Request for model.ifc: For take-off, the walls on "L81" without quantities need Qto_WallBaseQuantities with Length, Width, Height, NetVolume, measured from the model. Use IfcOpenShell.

First a look at what the model holds.

```python
import ifcopenshell
import ifcopenshell.util.element
import ifcopenshell.util.unit

model = ifcopenshell.open("model.ifc")
print(model.schema)
for unit_type in ("LENGTHUNIT", "AREAUNIT", "VOLUMEUNIT"):
    print(unit_type, ifcopenshell.util.unit.calculate_unit_scale(model, unit_type))
storey = next(s for s in model.by_type("IfcBuildingStorey") if s.Name == "L81")
walls = [e for e in ifcopenshell.util.element.get_decomposition(storey) if e.is_a("IfcWall")]
for e in sorted(walls, key=lambda e: e.id()):
    print(e.id(), e.is_a(), e.Name, list(ifcopenshell.util.element.get_psets(e, qtos_only=True)), sep=" | ")
```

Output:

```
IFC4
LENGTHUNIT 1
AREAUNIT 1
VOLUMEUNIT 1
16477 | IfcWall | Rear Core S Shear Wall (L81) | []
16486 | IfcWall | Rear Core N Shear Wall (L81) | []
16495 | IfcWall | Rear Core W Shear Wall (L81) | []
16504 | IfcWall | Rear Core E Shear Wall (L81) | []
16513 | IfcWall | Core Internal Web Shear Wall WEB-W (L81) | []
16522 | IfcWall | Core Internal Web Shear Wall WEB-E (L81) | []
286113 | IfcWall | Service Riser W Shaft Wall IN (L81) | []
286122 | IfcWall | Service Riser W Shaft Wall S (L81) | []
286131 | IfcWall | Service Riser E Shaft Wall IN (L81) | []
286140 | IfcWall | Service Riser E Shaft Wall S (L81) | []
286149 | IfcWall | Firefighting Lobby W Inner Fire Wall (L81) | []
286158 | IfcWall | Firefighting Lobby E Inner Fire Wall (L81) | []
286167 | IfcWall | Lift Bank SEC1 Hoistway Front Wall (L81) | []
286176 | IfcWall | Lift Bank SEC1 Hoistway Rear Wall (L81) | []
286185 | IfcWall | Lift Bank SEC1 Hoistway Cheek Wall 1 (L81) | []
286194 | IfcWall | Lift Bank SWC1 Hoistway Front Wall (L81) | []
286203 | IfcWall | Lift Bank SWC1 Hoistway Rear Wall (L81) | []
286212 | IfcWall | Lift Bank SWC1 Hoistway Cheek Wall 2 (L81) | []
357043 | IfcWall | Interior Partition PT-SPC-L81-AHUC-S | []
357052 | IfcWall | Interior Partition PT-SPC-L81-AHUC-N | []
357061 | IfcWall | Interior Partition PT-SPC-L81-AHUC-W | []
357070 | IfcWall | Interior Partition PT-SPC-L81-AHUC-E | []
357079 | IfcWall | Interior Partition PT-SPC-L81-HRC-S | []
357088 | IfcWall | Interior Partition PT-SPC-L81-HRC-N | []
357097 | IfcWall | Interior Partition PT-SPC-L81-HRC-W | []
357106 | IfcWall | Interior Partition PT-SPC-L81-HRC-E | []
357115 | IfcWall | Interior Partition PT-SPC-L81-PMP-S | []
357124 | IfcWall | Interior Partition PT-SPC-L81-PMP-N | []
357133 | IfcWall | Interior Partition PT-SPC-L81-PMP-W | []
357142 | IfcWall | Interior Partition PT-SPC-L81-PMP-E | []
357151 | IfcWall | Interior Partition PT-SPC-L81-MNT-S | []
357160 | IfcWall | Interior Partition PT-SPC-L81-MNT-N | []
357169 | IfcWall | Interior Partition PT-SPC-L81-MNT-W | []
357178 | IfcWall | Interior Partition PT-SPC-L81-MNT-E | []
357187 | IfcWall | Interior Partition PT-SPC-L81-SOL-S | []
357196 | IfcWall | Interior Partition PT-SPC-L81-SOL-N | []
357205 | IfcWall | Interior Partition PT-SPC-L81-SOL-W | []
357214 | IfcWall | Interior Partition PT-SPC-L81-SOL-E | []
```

```python
import ifcopenshell
import ifcopenshell.api.pset
import ifcopenshell.geom
import ifcopenshell.util.element
import ifcopenshell.util.shape
import ifcopenshell.util.unit

model = ifcopenshell.open("model.ifc")
unit_scale = ifcopenshell.util.unit.calculate_unit_scale(model)
volume_scale = ifcopenshell.util.unit.calculate_unit_scale(model, "VOLUMEUNIT")
settings = ifcopenshell.geom.settings()

storey = next(s for s in model.by_type("IfcBuildingStorey") if s.Name == "L81")
walls = [e for e in ifcopenshell.util.element.get_decomposition(storey) if e.is_a("IfcWall")]

for e in sorted(walls, key=lambda e: e.id()):
    if ifcopenshell.util.element.get_psets(e, qtos_only=True, should_inherit=False):
        continue
    # Geometry comes back in metres, in the element's own axes.
    shape = ifcopenshell.geom.create_shape(settings, e)
    values = {
        "Length": ifcopenshell.util.shape.get_x(shape.geometry) / unit_scale,
        "Width": ifcopenshell.util.shape.get_y(shape.geometry) / unit_scale,
        "Height": ifcopenshell.util.shape.get_z(shape.geometry) / unit_scale,
        "NetVolume": ifcopenshell.util.shape.get_volume(shape.geometry) / volume_scale,
    }
    qto = ifcopenshell.api.pset.add_qto(model, product=e, name="Qto_WallBaseQuantities")
    ifcopenshell.api.pset.edit_qto(model, qto=qto, properties=values)
    print(e.id(), {k: round(v, 3) for k, v in values.items()})

model.write("model-out.ifc")
```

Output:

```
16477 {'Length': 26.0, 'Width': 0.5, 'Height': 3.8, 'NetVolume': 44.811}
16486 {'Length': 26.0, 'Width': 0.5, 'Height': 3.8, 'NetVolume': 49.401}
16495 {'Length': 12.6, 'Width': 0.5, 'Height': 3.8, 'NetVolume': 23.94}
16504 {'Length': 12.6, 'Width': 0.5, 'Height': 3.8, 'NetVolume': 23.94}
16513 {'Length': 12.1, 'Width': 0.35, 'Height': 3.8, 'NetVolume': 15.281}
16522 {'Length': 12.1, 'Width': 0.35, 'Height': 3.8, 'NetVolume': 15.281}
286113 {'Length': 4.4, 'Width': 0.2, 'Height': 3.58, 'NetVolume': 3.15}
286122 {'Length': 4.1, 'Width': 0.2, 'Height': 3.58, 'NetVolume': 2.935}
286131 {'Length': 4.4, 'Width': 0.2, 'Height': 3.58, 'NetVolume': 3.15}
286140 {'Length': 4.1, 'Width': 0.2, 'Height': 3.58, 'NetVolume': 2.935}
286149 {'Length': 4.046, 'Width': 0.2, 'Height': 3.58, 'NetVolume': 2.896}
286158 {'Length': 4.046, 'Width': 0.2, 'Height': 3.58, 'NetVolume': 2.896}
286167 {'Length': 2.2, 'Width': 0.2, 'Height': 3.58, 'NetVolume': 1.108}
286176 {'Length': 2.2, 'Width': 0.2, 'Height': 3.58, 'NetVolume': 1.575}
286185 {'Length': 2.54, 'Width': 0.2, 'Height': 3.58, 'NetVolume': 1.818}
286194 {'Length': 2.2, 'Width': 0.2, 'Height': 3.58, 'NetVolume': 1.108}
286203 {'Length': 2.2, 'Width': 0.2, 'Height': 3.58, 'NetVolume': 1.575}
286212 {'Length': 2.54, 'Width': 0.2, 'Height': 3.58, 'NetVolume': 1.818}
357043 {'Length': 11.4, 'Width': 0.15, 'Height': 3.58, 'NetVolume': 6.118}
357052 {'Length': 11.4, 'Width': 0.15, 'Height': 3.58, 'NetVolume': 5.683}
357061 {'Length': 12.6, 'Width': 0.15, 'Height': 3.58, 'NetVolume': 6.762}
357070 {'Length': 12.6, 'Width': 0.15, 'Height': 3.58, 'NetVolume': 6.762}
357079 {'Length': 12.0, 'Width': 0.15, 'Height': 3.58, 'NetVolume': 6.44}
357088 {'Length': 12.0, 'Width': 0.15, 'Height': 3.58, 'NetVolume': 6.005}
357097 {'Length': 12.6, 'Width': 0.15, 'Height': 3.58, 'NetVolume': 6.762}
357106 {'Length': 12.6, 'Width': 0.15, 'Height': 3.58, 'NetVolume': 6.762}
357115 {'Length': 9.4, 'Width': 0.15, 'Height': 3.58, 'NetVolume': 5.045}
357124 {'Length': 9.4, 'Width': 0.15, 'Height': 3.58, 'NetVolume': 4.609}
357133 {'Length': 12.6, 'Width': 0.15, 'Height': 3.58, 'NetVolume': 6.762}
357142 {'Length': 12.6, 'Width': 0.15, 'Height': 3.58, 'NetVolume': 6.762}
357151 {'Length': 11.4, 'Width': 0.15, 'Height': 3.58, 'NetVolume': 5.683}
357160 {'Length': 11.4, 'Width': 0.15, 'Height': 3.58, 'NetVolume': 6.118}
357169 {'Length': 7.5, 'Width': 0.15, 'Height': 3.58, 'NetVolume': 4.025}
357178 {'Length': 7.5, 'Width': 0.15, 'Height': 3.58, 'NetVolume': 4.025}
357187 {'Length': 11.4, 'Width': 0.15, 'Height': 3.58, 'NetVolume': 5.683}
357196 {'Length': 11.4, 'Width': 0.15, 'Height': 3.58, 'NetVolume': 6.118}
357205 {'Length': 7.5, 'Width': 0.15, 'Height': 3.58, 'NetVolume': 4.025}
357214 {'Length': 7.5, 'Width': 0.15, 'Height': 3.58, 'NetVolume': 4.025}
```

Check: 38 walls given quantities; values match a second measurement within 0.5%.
